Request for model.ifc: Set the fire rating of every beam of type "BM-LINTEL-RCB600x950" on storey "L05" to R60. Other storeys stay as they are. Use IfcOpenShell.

First a look at what the model holds.

```python
import ifcopenshell
import ifcopenshell.util.element

model = ifcopenshell.open("model.ifc")
print(model.schema)
storey = next(s for s in model.by_type("IfcBuildingStorey") if s.Name == "L05")
beams = [e for e in ifcopenshell.util.element.get_decomposition(storey) if e.is_a("IfcBeam")]
seen = {}
for e in beams:
    element_type = ifcopenshell.util.element.get_type(e)
    key = (element_type.Name if element_type != e and element_type else None, ifcopenshell.util.element.get_pset(e, "Pset_BeamCommon", "FireRating"))
    seen[key] = seen.get(key, 0) + 1
for (name, value), count in sorted(seen.items(), key=str):
    print(count, "x", name, "|", value)
```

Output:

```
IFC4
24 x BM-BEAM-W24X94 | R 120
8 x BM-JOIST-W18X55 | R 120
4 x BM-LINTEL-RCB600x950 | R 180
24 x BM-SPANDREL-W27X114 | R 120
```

```python
import ifcopenshell
import ifcopenshell.api.pset
import ifcopenshell.util.element

model = ifcopenshell.open("model.ifc")

storey = next(s for s in model.by_type("IfcBuildingStorey") if s.Name == "L05")
beams = [e for e in ifcopenshell.util.element.get_decomposition(storey) if e.is_a("IfcBeam")]

count = 0
for e in beams:
    element_type = ifcopenshell.util.element.get_type(e)
    if element_type in (None, e) or element_type.Name != "BM-LINTEL-RCB600x950":
        continue
    found = ifcopenshell.util.element.get_pset(e, "Pset_BeamCommon", should_inherit=False)
    if found:
        pset = model.by_id(found["id"])
        if len(ifcopenshell.util.element.get_elements_by_pset(pset)) > 1:
            pset = ifcopenshell.api.pset.unshare_pset(model, products=[e], pset=pset)[0]
    else:
        pset = ifcopenshell.api.pset.add_pset(model, product=e, name="Pset_BeamCommon")
    ifcopenshell.api.pset.edit_pset(model, pset=pset, properties={"FireRating": "R60"})
    count += 1

print(count, "beams updated")

model.write("model-out.ifc")
```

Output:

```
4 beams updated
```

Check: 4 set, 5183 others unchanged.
